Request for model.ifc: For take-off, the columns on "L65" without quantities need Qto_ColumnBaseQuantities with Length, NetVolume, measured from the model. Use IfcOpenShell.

First a look at what the model holds.

```python
import ifcopenshell
import ifcopenshell.util.element
import ifcopenshell.util.unit

model = ifcopenshell.open("model.ifc")
print(model.schema)
for unit_type in ("LENGTHUNIT", "AREAUNIT", "VOLUMEUNIT"):
    print(unit_type, ifcopenshell.util.unit.calculate_unit_scale(model, unit_type))
storey = next(s for s in model.by_type("IfcBuildingStorey") if s.Name == "L65")
columns = [e for e in ifcopenshell.util.element.get_decomposition(storey) if e.is_a("IfcColumn")]
for e in sorted(columns, key=lambda e: e.id()):
    print(e.id(), e.is_a(), e.Name, list(ifcopenshell.util.element.get_psets(e, qtos_only=True)), sep=" | ")
```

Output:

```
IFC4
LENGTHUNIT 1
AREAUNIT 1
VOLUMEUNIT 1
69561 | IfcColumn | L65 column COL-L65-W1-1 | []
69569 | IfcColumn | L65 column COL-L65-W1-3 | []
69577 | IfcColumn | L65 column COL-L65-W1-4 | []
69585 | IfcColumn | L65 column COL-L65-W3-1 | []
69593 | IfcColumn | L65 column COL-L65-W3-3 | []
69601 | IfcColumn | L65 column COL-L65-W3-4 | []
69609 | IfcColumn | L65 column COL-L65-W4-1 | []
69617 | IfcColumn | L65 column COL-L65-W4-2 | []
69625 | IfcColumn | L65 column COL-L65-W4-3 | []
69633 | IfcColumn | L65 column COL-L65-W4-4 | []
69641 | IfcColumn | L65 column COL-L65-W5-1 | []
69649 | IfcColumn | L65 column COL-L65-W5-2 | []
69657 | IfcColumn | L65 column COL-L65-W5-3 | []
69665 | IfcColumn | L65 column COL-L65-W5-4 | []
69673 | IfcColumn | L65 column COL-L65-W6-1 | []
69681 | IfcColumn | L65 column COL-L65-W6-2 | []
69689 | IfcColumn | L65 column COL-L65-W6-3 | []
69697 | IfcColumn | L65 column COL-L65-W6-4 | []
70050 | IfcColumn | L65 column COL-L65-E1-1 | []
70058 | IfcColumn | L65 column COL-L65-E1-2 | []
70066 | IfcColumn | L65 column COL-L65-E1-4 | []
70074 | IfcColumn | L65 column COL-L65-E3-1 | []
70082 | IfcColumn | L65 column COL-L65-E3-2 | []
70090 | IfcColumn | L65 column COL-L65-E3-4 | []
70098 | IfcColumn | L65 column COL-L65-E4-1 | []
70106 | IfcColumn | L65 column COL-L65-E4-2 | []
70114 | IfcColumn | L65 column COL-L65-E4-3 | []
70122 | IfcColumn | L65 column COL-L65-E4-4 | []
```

```python
import ifcopenshell
import ifcopenshell.api.pset
import ifcopenshell.geom
import ifcopenshell.util.element
import ifcopenshell.util.shape
import ifcopenshell.util.unit

model = ifcopenshell.open("model.ifc")
unit_scale = ifcopenshell.util.unit.calculate_unit_scale(model)
volume_scale = ifcopenshell.util.unit.calculate_unit_scale(model, "VOLUMEUNIT")
settings = ifcopenshell.geom.settings()

storey = next(s for s in model.by_type("IfcBuildingStorey") if s.Name == "L65")
columns = [e for e in ifcopenshell.util.element.get_decomposition(storey) if e.is_a("IfcColumn")]

for e in sorted(columns, key=lambda e: e.id()):
    if ifcopenshell.util.element.get_psets(e, qtos_only=True, should_inherit=False):
        continue
    # Geometry comes back in metres, in the element's own axes.
    shape = ifcopenshell.geom.create_shape(settings, e)
    values = {
        "Length": ifcopenshell.util.shape.get_z(shape.geometry) / unit_scale,
        "NetVolume": ifcopenshell.util.shape.get_volume(shape.geometry) / volume_scale,
    }
    qto = ifcopenshell.api.pset.add_qto(model, product=e, name="Qto_ColumnBaseQuantities")
    ifcopenshell.api.pset.edit_qto(model, qto=qto, properties=values)
    print(e.id(), {k: round(v, 3) for k, v in values.items()})

model.write("model_rev.ifc")
```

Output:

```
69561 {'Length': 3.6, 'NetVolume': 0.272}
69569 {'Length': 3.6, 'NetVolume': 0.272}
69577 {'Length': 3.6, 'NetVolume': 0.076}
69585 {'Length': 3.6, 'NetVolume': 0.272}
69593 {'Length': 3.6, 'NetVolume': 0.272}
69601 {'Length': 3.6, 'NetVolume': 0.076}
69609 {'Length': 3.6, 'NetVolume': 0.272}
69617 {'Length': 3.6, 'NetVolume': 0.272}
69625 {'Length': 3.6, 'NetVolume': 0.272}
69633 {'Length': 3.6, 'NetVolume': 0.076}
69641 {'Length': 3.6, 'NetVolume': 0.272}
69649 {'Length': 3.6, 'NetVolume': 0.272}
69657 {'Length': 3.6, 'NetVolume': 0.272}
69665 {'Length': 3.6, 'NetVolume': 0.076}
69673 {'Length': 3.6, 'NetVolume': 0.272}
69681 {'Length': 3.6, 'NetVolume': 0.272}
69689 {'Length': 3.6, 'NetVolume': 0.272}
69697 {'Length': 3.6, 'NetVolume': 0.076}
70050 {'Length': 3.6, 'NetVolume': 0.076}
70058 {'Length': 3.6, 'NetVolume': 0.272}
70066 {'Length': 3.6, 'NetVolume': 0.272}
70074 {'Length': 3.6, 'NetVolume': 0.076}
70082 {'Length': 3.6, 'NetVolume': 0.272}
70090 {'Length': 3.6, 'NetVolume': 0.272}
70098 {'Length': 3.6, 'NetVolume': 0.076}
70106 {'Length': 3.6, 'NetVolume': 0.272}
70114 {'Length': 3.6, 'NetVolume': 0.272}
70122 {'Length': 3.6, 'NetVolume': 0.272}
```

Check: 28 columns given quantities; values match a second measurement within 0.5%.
